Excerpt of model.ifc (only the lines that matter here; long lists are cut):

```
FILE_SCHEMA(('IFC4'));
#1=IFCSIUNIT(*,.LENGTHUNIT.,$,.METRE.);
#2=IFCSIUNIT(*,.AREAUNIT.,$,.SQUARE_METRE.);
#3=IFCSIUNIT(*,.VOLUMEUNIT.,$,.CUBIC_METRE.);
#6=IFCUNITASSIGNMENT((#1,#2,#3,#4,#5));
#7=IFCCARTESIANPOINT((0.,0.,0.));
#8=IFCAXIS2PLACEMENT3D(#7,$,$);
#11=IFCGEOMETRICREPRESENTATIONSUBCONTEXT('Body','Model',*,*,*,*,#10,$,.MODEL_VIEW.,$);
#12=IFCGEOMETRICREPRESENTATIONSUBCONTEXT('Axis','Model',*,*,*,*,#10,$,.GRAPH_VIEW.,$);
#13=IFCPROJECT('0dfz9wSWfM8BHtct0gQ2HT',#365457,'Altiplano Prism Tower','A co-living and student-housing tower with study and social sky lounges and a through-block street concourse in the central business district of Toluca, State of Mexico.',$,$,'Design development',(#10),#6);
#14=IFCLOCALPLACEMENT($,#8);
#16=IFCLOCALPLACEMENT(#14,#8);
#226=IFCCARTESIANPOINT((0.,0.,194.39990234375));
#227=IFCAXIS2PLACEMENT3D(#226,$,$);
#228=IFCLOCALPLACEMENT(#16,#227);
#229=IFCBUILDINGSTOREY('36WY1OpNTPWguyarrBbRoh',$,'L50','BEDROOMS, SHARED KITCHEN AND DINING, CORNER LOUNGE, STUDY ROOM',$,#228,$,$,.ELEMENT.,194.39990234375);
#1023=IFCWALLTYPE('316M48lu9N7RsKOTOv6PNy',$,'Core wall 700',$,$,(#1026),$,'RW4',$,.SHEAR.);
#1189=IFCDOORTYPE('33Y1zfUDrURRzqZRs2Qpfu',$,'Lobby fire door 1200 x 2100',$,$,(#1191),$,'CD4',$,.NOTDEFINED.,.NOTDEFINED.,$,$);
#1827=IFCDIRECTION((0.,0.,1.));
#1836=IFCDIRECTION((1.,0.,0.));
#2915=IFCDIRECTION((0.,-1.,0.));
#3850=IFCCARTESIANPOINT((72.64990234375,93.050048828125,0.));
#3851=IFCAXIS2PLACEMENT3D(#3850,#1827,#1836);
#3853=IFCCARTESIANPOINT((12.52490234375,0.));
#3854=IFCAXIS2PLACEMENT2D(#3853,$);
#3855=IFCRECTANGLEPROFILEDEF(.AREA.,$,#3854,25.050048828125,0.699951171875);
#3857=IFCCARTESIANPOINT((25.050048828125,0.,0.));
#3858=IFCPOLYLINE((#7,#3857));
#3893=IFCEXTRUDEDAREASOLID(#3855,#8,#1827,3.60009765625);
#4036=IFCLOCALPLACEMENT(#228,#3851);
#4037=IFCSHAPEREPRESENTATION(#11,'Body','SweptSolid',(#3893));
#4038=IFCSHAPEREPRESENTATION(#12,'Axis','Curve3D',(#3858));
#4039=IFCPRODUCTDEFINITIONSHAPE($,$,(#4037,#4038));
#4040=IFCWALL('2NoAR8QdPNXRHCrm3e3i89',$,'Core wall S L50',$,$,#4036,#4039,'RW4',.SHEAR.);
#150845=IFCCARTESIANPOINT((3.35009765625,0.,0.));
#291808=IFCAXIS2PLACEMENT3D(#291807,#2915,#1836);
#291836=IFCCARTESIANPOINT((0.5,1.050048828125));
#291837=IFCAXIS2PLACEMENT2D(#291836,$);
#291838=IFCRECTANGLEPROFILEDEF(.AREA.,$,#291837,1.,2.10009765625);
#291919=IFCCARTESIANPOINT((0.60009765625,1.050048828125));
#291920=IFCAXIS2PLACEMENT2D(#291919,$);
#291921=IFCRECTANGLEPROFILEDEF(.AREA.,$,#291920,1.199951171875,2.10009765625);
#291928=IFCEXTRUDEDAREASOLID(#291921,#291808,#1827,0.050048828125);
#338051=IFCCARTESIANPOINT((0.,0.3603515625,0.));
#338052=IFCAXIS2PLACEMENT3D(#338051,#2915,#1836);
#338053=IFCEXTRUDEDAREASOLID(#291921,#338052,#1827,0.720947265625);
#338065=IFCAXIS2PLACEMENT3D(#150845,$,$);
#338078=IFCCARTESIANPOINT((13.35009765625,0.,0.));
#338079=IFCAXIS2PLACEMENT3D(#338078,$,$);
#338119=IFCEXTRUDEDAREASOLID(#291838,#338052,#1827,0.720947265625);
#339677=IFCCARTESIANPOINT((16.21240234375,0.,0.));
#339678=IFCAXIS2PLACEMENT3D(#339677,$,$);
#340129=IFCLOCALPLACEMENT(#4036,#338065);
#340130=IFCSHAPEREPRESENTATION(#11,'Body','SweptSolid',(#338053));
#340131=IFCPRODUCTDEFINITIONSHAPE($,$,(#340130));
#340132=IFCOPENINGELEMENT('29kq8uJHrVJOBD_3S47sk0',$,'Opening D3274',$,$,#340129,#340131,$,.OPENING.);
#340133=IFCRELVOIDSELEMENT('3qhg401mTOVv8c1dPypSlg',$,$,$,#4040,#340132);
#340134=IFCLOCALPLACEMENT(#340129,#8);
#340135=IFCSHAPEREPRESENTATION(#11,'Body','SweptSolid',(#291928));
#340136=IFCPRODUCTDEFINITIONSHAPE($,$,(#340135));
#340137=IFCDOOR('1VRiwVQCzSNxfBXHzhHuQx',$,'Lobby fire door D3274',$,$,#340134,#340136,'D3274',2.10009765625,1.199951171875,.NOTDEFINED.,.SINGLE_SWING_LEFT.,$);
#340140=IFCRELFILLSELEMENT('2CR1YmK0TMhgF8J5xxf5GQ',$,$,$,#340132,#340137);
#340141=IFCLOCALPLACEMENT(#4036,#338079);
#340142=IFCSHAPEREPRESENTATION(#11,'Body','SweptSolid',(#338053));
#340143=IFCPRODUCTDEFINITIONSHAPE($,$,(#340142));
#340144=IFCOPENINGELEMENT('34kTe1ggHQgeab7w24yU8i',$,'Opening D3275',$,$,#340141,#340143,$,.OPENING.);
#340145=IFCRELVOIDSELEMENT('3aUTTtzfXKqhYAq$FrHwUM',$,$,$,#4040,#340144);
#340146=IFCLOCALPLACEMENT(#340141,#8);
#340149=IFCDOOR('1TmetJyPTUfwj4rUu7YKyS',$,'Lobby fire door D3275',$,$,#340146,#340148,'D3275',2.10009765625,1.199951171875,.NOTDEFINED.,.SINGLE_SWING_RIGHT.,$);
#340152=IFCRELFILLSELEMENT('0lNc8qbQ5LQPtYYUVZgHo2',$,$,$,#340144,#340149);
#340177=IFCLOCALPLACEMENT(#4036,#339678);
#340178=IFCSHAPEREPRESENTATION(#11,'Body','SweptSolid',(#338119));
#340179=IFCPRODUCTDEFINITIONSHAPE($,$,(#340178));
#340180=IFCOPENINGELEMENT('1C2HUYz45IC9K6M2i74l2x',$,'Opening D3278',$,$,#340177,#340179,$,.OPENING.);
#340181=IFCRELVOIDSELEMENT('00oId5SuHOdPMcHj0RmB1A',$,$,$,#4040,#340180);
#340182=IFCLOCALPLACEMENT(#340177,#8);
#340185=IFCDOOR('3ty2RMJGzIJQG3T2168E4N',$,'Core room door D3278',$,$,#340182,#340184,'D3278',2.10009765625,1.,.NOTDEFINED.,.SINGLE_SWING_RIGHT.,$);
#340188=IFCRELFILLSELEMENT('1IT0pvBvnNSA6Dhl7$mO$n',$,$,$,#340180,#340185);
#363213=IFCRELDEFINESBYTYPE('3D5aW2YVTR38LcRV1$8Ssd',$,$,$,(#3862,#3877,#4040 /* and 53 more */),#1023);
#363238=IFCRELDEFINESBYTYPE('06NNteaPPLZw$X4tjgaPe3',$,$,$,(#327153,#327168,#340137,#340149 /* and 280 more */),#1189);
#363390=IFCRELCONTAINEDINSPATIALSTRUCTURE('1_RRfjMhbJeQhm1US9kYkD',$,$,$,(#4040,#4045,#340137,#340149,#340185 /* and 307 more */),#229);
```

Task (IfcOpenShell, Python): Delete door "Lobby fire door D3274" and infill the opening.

```python
import ifcopenshell
import ifcopenshell.api.feature
import ifcopenshell.api.root
import ifcopenshell.geom
import ifcopenshell.util.shape

model = ifcopenshell.open("model.ifc")
settings = ifcopenshell.geom.settings()


def volume(element):
    """Net volume in cubic metres, openings subtracted."""
    shape = ifcopenshell.geom.create_shape(settings, element)
    return ifcopenshell.util.shape.get_volume(shape.geometry)


door = model.by_id(340137)
opening = door.FillsVoids[0].RelatingOpeningElement
wall = opening.VoidsElements[0].RelatingBuildingElement
before = volume(wall)

ifcopenshell.api.root.remove_product(model, product=door)
ifcopenshell.api.feature.remove_feature(model, feature=opening)

after = volume(wall)

print(f"wall volume {before:.3f} -> {after:.3f} m3")

model.write("model_edited.ifc")
```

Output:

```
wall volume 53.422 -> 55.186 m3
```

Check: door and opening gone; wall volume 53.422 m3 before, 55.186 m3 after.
